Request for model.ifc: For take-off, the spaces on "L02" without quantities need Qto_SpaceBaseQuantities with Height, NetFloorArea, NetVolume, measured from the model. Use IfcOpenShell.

First a look at what the model holds.

```python
import ifcopenshell
import ifcopenshell.util.element
import ifcopenshell.util.unit

model = ifcopenshell.open("model.ifc")
print(model.schema)
for unit_type in ("LENGTHUNIT", "AREAUNIT", "VOLUMEUNIT"):
    print(unit_type, ifcopenshell.util.unit.calculate_unit_scale(model, unit_type))
storey = next(s for s in model.by_type("IfcBuildingStorey") if s.Name == "L02")
spaces = [e for e in ifcopenshell.util.element.get_decomposition(storey) if e.is_a("IfcSpace")]
for e in sorted(spaces, key=lambda e: e.id()):
    print(e.id(), e.is_a(), e.Name, list(ifcopenshell.util.element.get_psets(e, qtos_only=True)), sep=" | ")
```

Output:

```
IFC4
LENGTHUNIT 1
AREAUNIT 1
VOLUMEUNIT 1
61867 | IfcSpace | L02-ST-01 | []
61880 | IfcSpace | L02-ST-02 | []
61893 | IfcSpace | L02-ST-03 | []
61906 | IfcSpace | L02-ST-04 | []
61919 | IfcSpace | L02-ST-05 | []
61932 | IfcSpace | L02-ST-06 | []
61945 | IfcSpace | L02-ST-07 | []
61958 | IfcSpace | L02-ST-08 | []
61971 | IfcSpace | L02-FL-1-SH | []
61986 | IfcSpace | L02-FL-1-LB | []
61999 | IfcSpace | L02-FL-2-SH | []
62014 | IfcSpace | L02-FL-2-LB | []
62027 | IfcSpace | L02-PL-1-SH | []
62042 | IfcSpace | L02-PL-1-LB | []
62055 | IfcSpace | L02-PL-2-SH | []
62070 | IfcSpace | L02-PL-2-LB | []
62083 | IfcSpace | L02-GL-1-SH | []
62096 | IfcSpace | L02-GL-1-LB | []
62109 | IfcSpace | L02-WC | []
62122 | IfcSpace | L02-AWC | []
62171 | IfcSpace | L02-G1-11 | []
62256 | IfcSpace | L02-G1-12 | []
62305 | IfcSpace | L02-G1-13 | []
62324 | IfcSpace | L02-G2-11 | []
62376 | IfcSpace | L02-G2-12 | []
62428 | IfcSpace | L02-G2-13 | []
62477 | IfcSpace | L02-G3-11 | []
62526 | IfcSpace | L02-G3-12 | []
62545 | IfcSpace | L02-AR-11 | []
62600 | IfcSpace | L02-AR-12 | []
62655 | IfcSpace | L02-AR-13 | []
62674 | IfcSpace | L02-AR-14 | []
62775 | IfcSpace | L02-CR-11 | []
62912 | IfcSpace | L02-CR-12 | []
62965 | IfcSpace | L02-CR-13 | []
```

```python
import ifcopenshell
import ifcopenshell.api.pset
import ifcopenshell.geom
import ifcopenshell.util.element
import ifcopenshell.util.shape
import ifcopenshell.util.unit

model = ifcopenshell.open("model.ifc")
unit_scale = ifcopenshell.util.unit.calculate_unit_scale(model)
area_scale = ifcopenshell.util.unit.calculate_unit_scale(model, "AREAUNIT")
volume_scale = ifcopenshell.util.unit.calculate_unit_scale(model, "VOLUMEUNIT")
settings = ifcopenshell.geom.settings()

storey = next(s for s in model.by_type("IfcBuildingStorey") if s.Name == "L02")
spaces = [e for e in ifcopenshell.util.element.get_decomposition(storey) if e.is_a("IfcSpace")]

for e in sorted(spaces, key=lambda e: e.id()):
    if ifcopenshell.util.element.get_psets(e, qtos_only=True, should_inherit=False):
        continue
    # Geometry comes back in metres, in the element's own axes.
    shape = ifcopenshell.geom.create_shape(settings, e)
    values = {
        "Height": ifcopenshell.util.shape.get_z(shape.geometry) / unit_scale,
        "NetFloorArea": ifcopenshell.util.shape.get_footprint_area(shape.geometry) / area_scale,
        "NetVolume": ifcopenshell.util.shape.get_volume(shape.geometry) / volume_scale,
    }
    qto = ifcopenshell.api.pset.add_qto(model, product=e, name="Qto_SpaceBaseQuantities")
    ifcopenshell.api.pset.edit_qto(model, qto=qto, properties=values)
    print(e.id(), {k: round(v, 3) for k, v in values.items()})

model.write("model_rev.ifc")
```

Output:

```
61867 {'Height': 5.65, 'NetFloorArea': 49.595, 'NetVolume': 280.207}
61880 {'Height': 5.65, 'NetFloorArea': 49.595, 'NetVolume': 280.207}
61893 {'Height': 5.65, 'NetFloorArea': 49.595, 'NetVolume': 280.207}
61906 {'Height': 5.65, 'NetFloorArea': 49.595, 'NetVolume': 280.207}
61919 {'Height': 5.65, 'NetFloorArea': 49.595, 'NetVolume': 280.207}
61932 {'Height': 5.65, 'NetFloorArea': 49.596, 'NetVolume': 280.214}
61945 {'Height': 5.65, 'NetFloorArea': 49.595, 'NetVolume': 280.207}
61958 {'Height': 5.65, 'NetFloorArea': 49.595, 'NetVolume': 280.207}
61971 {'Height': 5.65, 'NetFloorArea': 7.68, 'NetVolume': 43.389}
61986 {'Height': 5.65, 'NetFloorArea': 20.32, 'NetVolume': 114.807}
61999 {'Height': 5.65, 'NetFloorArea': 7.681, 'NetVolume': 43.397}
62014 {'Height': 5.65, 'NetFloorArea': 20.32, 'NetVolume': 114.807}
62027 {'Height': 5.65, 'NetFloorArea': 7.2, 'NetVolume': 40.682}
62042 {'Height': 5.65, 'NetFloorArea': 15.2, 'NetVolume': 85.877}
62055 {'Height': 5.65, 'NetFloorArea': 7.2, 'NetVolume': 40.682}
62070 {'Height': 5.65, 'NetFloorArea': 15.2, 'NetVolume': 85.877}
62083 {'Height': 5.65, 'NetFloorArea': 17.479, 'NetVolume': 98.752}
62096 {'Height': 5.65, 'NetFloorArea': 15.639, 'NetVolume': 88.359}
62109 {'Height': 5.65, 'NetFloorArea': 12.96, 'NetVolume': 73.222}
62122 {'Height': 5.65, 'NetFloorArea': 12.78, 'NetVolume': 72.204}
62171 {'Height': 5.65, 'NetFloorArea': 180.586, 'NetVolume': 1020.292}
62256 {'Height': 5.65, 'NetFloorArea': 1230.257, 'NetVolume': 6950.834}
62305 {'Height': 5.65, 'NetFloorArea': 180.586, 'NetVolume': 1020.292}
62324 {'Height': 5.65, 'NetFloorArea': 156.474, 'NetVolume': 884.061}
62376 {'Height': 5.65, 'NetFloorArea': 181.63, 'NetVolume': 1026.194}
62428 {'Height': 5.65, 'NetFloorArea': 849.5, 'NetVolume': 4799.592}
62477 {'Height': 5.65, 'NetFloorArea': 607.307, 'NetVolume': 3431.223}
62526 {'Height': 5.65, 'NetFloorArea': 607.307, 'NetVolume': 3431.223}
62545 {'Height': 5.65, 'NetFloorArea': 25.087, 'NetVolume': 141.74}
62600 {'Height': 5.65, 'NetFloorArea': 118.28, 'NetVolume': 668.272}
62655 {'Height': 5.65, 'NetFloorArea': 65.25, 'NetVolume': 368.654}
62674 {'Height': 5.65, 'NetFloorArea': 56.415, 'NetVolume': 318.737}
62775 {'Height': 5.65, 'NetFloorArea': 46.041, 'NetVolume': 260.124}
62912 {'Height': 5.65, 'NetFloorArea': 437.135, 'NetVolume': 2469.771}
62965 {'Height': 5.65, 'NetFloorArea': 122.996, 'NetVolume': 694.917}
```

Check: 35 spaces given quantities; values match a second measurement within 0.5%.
